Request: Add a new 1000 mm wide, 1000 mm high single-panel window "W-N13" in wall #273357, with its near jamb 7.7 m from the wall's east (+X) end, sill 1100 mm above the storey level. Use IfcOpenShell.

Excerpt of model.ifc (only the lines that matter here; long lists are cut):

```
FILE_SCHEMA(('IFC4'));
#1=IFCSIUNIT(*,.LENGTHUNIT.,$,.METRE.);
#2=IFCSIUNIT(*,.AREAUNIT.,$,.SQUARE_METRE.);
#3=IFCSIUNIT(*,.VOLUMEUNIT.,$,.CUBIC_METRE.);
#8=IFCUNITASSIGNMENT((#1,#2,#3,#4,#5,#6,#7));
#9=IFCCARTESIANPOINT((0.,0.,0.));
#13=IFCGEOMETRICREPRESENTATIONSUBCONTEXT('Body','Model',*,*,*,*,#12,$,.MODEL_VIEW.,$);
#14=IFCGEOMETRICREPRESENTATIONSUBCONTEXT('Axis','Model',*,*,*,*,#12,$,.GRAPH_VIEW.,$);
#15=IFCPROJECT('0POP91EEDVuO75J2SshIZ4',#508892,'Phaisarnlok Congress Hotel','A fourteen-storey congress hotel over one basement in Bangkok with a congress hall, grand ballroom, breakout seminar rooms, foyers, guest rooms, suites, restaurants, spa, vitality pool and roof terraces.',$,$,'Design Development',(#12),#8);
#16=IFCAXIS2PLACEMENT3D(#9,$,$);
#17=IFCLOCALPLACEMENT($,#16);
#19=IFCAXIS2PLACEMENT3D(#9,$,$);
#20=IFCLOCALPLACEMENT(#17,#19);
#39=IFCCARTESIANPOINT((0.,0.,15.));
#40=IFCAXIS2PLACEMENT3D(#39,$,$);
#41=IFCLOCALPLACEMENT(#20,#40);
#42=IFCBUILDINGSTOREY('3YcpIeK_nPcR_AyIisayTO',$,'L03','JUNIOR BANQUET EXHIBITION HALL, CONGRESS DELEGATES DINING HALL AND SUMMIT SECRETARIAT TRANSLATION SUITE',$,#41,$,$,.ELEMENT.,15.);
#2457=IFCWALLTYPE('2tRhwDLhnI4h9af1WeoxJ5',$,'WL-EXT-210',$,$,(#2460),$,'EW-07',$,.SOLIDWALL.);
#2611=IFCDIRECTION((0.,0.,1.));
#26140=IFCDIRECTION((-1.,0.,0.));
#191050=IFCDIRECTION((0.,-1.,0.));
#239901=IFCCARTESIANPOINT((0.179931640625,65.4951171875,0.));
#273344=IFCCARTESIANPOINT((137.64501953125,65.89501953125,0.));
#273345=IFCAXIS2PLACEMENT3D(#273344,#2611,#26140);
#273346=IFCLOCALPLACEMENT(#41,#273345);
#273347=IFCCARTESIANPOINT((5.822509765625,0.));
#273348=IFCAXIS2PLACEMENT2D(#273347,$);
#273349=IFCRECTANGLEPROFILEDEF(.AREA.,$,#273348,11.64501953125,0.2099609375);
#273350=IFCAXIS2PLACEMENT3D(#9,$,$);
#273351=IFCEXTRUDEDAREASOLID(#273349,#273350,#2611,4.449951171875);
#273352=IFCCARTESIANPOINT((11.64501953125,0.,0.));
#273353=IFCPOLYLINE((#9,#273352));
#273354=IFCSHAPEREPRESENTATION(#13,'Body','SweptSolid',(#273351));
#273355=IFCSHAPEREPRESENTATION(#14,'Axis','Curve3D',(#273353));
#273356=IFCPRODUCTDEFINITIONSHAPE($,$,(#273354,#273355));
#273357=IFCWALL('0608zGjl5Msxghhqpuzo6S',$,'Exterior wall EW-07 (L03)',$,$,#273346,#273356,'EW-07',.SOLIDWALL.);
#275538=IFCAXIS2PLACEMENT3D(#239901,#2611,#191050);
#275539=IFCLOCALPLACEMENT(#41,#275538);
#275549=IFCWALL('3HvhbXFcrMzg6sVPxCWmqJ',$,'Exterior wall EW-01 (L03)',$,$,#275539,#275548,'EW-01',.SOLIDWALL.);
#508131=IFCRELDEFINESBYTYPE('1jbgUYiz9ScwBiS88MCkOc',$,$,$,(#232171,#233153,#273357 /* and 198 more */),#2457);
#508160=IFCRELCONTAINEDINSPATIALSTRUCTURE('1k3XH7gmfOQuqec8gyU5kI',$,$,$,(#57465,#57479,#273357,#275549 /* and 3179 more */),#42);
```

```python
import numpy as np
import ifcopenshell
import ifcopenshell.api.feature
import ifcopenshell.api.geometry
import ifcopenshell.api.root
import ifcopenshell.api.spatial
import ifcopenshell.geom
import ifcopenshell.util.element
import ifcopenshell.util.placement
import ifcopenshell.util.representation
import ifcopenshell.util.shape
import ifcopenshell.util.unit

model = ifcopenshell.open("model.ifc")
unit_scale = ifcopenshell.util.unit.calculate_unit_scale(model)
settings = ifcopenshell.geom.settings()


def volume(element):
    """Net volume in cubic metres, openings subtracted."""
    shape = ifcopenshell.geom.create_shape(settings, element)
    return ifcopenshell.util.shape.get_volume(shape.geometry)


wall = model.by_guid("0608zGjl5Msxghhqpuzo6S")
storey = ifcopenshell.util.element.get_container(wall, ifc_class="IfcBuildingStorey")
context = ifcopenshell.util.representation.get_context(model, "Model", "Body", "MODEL_VIEW")
before = volume(wall)

width, height, from_end, sill = 1, 1, 7.7, 1.1  # metres

# The wall runs along its own X axis, and the end named is its -X end.
wall_shape = ifcopenshell.geom.create_shape(settings, wall)
x, y, z = ifcopenshell.util.shape.get_vertices(wall_shape.geometry).T
start = x.min() + from_end
face, thickness = float(y.min()), float(y.max() - y.min())
wall_matrix = ifcopenshell.util.placement.get_local_placement(wall.ObjectPlacement)
level = ifcopenshell.util.placement.get_local_placement(storey.ObjectPlacement)[2, 3]


def in_wall(x, y):
    """Placement at x, y metres in the wall's axes, at sill height."""
    matrix = wall_matrix.copy()
    matrix[:, 3] = wall_matrix @ np.array([x / unit_scale, y / unit_scale, 0.0, 1.0])
    matrix[2, 3] = level + sill / unit_scale
    return matrix


# Opening: a box that overshoots both wall faces by 50 mm.
opening = ifcopenshell.api.root.create_entity(model, ifc_class="IfcOpeningElement", predefined_type="OPENING")
box = ifcopenshell.api.geometry.add_wall_representation(
    model, context=context, length=width, height=height, thickness=thickness + 0.1
)
ifcopenshell.api.geometry.assign_representation(model, product=opening, representation=box)
ifcopenshell.api.geometry.edit_object_placement(model, product=opening, matrix=in_wall(start, face - 0.05), is_si=False)
ifcopenshell.api.feature.add_feature(model, feature=opening, element=wall)

window = ifcopenshell.api.root.create_entity(model, ifc_class="IfcWindow", name="W-N13", predefined_type="WINDOW")
window.OverallWidth, window.OverallHeight = width / unit_scale, height / unit_scale
window.PartitioningType = "SINGLE_PANEL"
body = ifcopenshell.api.geometry.add_window_representation(
    model,
    context=context,
    overall_width=window.OverallWidth,
    overall_height=window.OverallHeight,
    partition_type="SINGLE_PANEL",
)
ifcopenshell.api.geometry.assign_representation(model, product=window, representation=body)
ifcopenshell.api.spatial.assign_container(model, products=[window], relating_structure=storey)
ifcopenshell.api.feature.add_filling(model, opening=opening, element=window)

# Centre the window in the wall's thickness.
ifcopenshell.api.geometry.edit_object_placement(model, product=window, matrix=in_wall(start, face), is_si=False)
window_shape = ifcopenshell.geom.create_shape(settings, window)
depth = ifcopenshell.util.shape.get_vertices(window_shape.geometry)[:, 1]
offset = face + thickness / 2 - (depth.min() + depth.max()) / 2
ifcopenshell.api.geometry.edit_object_placement(model, product=window, matrix=in_wall(start, offset), is_si=False)

after = volume(wall)

print(f"wall volume {before:.3f} -> {after:.3f} m3")

model.write("model_rev.ifc")
```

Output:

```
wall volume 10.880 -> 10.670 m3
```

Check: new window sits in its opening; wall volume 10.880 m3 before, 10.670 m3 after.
